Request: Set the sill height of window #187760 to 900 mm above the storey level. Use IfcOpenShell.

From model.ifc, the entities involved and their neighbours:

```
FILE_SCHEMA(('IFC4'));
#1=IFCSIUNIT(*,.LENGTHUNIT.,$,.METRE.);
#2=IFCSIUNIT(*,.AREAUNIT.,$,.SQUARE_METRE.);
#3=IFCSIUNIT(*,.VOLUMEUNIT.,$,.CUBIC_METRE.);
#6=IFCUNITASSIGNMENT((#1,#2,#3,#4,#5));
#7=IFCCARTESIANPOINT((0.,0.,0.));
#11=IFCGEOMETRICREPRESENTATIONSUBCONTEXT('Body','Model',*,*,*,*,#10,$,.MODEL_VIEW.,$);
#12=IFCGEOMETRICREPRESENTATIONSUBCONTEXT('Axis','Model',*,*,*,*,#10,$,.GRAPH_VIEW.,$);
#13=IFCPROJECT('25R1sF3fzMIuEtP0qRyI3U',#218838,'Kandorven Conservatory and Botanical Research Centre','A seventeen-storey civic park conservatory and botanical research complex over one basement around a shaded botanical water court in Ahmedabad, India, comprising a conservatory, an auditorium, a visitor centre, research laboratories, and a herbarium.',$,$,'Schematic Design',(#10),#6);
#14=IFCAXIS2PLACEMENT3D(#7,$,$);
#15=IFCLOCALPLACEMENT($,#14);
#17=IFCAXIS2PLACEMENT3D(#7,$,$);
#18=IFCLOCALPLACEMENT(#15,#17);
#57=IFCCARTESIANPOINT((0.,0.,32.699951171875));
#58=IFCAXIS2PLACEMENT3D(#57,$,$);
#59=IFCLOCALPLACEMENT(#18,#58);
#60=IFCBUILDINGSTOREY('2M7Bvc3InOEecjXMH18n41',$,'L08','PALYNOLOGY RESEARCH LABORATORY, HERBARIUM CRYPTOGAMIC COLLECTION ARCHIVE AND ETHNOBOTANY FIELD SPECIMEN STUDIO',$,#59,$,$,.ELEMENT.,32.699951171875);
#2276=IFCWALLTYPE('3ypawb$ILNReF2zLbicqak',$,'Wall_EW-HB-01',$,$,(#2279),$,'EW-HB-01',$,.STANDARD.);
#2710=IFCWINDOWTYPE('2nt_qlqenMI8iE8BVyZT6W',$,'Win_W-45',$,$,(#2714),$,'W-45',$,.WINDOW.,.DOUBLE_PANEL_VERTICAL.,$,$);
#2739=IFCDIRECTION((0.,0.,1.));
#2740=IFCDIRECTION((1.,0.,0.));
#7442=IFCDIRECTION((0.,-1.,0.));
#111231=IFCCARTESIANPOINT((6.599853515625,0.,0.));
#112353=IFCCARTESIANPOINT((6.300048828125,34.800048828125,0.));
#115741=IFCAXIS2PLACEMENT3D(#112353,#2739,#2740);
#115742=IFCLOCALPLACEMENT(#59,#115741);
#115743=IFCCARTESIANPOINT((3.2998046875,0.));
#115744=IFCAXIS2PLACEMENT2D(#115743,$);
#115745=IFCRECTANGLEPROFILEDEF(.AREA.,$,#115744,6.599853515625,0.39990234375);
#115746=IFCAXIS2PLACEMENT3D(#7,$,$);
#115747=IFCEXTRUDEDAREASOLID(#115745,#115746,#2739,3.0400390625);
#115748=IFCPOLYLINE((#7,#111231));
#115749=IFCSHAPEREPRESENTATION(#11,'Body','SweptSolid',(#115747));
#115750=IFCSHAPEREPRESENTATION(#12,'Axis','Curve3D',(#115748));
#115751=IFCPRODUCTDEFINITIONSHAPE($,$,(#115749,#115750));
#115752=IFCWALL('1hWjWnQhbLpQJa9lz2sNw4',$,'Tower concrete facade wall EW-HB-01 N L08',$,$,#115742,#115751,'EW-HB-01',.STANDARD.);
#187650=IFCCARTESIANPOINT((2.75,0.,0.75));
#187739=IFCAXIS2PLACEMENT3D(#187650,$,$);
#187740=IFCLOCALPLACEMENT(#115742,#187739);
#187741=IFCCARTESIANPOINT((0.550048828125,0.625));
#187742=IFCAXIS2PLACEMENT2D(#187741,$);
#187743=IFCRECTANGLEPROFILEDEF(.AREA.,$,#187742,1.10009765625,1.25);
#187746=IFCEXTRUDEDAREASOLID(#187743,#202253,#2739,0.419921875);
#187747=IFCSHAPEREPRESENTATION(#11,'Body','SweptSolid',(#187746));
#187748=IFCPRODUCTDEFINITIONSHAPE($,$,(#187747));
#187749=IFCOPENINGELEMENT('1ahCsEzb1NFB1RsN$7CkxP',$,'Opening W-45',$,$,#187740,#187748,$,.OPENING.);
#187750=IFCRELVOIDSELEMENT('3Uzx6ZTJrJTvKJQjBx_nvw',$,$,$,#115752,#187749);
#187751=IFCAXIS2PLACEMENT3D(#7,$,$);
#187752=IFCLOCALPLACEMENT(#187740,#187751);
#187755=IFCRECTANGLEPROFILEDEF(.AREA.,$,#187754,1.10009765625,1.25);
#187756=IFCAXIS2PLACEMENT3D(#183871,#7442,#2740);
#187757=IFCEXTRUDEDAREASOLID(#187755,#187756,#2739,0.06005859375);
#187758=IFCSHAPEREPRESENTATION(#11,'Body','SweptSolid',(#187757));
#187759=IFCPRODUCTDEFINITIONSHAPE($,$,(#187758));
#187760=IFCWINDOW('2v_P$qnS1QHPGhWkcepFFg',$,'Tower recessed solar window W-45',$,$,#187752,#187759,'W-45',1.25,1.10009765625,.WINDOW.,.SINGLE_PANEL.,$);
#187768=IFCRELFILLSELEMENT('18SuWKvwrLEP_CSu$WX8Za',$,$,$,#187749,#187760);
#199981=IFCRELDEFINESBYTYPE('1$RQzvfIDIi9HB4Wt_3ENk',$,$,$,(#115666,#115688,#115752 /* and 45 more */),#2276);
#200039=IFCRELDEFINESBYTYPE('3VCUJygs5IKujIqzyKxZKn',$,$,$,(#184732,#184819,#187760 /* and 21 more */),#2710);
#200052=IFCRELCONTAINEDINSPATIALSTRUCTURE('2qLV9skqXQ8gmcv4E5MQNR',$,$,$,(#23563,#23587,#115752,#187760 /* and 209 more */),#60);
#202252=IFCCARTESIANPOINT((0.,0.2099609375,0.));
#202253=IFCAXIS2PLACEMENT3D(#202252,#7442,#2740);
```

```python
import numpy as np
import ifcopenshell
import ifcopenshell.api.geometry
import ifcopenshell.geom
import ifcopenshell.util.element
import ifcopenshell.util.placement
import ifcopenshell.util.shape
import ifcopenshell.util.unit

model = ifcopenshell.open("model.ifc")
unit_scale = ifcopenshell.util.unit.calculate_unit_scale(model)

window = model.by_id(187760)
opening = window.FillsVoids[0].RelatingOpeningElement
storey = ifcopenshell.util.element.get_container(window, ifc_class="IfcBuildingStorey")
level = ifcopenshell.util.placement.get_local_placement(storey.ObjectPlacement)[2, 3]

# The opening's origin need not be at the sill, so measure its lowest point.
shape = ifcopenshell.geom.create_shape(ifcopenshell.geom.settings(), opening)
bottom = ifcopenshell.util.shape.get_shape_bottom_elevation(shape, shape.geometry) / unit_scale
dz = level + 0.9 / unit_scale - bottom

shift = np.array([0.0, 0.0, dz])
# The window is placed relative to its opening, so it follows when the opening moves.
matrix = ifcopenshell.util.placement.get_local_placement(opening.ObjectPlacement)
matrix[:3, 3] += shift
ifcopenshell.api.geometry.edit_object_placement(
    model, product=opening, matrix=matrix, is_si=False, should_transform_children=True
)

print(f"moved by {dz * unit_scale:+.3f} m")

model.write("model_rev.ifc")
```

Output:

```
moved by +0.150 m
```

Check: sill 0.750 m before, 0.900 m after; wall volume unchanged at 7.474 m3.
